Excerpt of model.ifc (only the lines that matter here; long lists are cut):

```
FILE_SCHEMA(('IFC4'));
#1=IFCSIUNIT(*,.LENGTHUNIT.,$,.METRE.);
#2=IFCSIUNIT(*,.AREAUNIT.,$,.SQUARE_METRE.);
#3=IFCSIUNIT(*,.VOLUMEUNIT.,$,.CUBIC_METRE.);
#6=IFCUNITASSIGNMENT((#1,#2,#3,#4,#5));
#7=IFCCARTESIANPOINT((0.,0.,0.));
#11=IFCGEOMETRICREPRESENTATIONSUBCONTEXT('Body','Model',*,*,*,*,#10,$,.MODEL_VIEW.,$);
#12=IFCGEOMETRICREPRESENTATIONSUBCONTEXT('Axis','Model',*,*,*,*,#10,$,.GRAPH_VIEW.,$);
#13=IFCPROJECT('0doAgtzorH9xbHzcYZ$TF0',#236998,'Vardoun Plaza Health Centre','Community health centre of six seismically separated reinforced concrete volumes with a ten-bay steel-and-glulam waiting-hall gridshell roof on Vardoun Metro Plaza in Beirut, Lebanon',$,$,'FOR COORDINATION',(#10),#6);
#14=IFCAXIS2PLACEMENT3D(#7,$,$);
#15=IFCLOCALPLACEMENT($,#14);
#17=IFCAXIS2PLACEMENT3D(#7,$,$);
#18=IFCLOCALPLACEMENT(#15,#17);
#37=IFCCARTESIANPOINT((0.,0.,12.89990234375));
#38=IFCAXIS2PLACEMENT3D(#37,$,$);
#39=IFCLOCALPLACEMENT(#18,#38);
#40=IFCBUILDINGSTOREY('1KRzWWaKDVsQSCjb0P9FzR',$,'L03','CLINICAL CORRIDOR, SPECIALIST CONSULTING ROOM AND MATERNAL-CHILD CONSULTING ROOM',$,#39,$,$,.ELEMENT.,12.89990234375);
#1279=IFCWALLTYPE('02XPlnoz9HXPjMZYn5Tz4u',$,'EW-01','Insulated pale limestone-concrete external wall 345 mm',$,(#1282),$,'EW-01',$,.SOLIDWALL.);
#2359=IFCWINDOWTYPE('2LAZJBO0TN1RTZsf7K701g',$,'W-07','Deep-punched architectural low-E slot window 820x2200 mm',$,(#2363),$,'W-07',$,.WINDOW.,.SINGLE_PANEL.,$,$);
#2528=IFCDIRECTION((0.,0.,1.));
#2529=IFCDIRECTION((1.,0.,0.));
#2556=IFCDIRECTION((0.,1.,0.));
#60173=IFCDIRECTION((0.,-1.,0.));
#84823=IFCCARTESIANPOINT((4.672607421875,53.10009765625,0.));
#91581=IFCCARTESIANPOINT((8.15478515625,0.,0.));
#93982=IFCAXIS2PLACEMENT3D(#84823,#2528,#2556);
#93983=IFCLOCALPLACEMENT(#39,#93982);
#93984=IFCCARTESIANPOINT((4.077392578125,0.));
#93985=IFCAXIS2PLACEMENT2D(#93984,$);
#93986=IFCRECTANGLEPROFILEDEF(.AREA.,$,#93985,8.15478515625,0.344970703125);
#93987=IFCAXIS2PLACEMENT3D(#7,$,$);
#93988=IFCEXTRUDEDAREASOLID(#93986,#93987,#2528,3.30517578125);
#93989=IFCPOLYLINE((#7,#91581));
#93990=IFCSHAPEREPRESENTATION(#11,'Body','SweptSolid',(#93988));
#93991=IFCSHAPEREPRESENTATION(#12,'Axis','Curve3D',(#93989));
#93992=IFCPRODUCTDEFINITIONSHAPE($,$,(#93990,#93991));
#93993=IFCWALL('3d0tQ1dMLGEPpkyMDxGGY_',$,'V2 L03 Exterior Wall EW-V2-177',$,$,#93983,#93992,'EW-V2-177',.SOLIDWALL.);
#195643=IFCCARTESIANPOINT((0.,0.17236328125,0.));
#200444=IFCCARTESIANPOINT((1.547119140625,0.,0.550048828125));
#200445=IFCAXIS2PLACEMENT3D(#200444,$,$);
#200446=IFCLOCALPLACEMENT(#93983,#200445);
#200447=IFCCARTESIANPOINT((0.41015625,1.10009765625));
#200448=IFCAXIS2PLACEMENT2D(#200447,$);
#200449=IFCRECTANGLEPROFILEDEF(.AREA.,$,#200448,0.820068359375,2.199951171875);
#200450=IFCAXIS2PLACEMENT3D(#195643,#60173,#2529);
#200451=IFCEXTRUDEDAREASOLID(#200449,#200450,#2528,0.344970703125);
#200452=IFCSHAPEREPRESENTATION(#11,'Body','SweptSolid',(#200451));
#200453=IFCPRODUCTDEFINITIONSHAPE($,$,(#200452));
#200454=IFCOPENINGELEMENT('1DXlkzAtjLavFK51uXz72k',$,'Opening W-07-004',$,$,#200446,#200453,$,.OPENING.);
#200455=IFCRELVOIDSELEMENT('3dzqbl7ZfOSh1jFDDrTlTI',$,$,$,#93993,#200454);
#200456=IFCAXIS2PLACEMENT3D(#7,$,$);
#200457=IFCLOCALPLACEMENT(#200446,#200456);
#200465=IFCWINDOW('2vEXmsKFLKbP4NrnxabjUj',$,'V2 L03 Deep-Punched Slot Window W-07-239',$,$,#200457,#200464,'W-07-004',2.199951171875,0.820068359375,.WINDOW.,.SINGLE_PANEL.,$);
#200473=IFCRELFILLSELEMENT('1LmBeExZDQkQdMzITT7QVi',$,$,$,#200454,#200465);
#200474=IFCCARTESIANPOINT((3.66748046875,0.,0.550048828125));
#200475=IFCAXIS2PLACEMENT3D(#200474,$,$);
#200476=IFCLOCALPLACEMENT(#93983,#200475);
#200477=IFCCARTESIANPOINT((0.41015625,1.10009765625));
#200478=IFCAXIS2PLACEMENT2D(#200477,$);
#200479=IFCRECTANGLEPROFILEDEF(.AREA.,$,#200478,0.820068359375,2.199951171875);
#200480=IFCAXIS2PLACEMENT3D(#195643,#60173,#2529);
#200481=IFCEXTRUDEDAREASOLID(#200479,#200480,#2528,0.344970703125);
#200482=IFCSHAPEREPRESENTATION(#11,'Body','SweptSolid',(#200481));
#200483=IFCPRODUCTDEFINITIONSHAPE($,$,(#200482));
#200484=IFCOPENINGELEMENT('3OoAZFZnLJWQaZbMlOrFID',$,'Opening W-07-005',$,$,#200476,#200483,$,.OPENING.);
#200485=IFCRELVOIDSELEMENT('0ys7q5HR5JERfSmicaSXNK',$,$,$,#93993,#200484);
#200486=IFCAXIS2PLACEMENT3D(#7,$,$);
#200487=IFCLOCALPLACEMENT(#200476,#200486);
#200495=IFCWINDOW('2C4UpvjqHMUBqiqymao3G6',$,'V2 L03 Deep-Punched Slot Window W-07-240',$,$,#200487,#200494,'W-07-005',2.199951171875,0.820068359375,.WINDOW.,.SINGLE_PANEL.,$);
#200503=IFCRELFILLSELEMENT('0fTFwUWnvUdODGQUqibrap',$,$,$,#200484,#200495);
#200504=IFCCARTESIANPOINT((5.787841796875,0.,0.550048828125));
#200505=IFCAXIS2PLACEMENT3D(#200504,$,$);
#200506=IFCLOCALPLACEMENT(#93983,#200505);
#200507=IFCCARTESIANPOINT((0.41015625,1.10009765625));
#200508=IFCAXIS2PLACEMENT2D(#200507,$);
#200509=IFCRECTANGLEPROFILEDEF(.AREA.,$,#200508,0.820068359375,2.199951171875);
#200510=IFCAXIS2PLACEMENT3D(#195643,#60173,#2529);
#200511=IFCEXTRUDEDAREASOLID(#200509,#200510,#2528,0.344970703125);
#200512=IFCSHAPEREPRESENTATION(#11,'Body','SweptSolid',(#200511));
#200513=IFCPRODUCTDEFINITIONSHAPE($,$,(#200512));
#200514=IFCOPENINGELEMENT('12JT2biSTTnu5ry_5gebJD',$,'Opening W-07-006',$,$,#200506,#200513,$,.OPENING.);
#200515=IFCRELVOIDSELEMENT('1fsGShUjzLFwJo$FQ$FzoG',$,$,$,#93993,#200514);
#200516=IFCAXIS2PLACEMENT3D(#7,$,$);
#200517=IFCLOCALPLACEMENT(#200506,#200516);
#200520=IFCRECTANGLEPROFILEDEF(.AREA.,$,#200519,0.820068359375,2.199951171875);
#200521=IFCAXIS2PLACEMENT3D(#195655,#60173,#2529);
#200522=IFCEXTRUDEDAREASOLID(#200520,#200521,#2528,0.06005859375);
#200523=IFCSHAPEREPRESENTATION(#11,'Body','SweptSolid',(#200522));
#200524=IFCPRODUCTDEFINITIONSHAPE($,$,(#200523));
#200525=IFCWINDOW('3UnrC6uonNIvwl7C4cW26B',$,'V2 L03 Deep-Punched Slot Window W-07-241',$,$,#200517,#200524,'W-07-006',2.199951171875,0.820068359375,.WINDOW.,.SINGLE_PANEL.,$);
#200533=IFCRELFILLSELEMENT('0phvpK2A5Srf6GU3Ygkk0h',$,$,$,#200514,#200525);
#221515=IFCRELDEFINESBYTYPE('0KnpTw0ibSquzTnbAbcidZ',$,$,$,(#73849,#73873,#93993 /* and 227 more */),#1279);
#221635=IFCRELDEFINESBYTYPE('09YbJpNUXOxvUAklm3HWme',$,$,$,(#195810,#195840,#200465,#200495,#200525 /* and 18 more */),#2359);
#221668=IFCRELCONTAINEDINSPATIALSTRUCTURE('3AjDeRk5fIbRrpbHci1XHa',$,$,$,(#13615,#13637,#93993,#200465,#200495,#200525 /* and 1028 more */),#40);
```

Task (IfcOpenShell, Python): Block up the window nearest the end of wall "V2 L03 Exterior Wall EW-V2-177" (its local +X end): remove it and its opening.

```python
import ifcopenshell
import ifcopenshell.api.feature
import ifcopenshell.api.root
import ifcopenshell.geom
import ifcopenshell.util.shape

model = ifcopenshell.open("model.ifc")
settings = ifcopenshell.geom.settings()


def volume(element):
    """Net volume in cubic metres, openings subtracted."""
    shape = ifcopenshell.geom.create_shape(settings, element)
    return ifcopenshell.util.shape.get_volume(shape.geometry)


window = model.by_id(200525)
opening = window.FillsVoids[0].RelatingOpeningElement
wall = opening.VoidsElements[0].RelatingBuildingElement
before = volume(wall)

ifcopenshell.api.root.remove_product(model, product=window)
ifcopenshell.api.feature.remove_feature(model, feature=opening)

after = volume(wall)

print(f"wall volume {before:.3f} -> {after:.3f} m3")

model.write("model-out.ifc")
```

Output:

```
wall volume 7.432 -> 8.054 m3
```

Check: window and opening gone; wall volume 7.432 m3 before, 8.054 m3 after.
